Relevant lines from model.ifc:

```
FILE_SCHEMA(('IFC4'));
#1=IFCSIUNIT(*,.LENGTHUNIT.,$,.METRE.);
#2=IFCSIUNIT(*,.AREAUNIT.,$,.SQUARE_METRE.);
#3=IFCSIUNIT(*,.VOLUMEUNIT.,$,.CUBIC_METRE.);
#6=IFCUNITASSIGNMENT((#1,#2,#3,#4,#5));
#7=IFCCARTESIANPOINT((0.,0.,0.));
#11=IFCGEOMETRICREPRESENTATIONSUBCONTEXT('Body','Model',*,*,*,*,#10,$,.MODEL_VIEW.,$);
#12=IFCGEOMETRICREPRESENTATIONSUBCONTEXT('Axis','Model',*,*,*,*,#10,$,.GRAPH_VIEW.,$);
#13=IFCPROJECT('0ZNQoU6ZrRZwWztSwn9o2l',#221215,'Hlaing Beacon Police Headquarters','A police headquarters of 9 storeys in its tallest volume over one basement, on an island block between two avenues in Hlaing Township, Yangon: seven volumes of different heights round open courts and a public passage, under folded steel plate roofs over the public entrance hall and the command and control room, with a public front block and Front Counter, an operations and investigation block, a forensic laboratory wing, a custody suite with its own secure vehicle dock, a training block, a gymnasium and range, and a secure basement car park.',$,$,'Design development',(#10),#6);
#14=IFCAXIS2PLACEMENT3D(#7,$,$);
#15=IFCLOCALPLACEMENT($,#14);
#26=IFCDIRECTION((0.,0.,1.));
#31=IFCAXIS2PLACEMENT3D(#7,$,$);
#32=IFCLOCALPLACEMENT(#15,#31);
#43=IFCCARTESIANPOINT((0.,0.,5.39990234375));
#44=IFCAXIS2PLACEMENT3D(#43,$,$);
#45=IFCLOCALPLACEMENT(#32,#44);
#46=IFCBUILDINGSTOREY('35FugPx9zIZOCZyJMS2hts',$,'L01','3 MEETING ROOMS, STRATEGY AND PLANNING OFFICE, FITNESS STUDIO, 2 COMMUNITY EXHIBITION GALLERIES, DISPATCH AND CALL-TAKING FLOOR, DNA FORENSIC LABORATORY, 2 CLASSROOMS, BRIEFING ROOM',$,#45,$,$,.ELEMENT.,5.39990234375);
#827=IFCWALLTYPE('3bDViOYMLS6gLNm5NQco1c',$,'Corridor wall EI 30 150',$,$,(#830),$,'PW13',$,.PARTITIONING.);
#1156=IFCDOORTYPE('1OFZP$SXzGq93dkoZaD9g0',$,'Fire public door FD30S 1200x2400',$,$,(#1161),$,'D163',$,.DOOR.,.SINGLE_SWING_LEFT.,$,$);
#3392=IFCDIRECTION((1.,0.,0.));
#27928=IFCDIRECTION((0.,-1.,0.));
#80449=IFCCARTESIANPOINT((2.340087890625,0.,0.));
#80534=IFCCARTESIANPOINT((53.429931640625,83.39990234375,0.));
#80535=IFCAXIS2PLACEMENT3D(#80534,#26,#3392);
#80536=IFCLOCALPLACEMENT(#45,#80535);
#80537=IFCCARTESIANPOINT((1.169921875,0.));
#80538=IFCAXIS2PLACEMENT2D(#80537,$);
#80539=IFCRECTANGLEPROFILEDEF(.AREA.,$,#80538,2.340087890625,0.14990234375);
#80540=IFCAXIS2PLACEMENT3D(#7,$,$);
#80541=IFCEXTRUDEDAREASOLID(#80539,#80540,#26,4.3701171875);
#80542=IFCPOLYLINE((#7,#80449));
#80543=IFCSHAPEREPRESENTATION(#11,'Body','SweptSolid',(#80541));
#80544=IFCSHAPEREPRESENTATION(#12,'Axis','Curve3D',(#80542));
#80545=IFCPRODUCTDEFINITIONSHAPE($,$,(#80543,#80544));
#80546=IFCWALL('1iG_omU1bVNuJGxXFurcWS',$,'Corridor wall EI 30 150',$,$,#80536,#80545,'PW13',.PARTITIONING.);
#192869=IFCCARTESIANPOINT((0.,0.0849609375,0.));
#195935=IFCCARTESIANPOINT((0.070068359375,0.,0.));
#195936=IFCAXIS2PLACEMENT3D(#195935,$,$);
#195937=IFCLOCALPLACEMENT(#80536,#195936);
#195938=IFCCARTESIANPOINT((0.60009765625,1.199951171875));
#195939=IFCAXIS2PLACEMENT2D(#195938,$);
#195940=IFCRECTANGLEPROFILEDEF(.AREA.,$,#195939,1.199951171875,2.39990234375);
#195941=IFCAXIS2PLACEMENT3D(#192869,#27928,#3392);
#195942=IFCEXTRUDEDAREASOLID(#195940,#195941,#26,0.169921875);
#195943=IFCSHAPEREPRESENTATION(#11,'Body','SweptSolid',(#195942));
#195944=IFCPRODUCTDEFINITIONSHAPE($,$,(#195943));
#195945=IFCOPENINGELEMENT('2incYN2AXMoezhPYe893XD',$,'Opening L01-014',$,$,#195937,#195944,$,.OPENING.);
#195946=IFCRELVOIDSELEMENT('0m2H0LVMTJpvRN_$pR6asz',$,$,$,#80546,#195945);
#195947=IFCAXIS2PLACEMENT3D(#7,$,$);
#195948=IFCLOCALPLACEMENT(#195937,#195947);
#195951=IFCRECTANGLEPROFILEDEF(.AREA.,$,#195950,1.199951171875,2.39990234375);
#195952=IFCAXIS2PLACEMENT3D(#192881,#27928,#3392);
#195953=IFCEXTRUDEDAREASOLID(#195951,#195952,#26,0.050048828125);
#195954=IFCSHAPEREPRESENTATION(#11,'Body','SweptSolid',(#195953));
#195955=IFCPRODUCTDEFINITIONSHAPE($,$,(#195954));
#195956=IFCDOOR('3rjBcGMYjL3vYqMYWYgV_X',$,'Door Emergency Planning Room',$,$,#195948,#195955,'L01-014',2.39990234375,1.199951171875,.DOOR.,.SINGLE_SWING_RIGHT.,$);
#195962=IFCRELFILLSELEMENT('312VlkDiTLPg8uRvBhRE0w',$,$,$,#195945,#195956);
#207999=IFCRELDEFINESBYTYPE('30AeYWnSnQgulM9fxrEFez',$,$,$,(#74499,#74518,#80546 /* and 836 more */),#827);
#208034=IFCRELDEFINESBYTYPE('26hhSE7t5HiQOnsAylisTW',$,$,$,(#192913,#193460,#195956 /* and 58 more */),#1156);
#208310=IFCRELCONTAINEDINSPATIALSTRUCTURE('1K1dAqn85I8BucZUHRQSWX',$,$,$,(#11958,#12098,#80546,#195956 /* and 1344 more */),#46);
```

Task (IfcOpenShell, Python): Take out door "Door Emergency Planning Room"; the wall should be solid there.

```python
import ifcopenshell
import ifcopenshell.api.feature
import ifcopenshell.api.root
import ifcopenshell.geom
import ifcopenshell.util.shape

model = ifcopenshell.open("model.ifc")
settings = ifcopenshell.geom.settings()


def volume(element):
    """Net volume in cubic metres, openings subtracted."""
    shape = ifcopenshell.geom.create_shape(settings, element)
    return ifcopenshell.util.shape.get_volume(shape.geometry)


door = model.by_guid("3rjBcGMYjL3vYqMYWYgV_X")
opening = door.FillsVoids[0].RelatingOpeningElement
wall = opening.VoidsElements[0].RelatingBuildingElement
before = volume(wall)

ifcopenshell.api.root.remove_product(model, product=door)
ifcopenshell.api.feature.remove_feature(model, feature=opening)

after = volume(wall)

print(f"wall volume {before:.3f} -> {after:.3f} m3")

model.write("model_edited.ifc")
```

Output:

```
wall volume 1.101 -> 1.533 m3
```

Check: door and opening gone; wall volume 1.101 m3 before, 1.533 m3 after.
